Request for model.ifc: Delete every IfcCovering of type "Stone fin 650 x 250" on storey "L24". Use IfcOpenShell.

First a look at what the model holds.

```python
import ifcopenshell
import ifcopenshell.util.element

model = ifcopenshell.open("model.ifc")
print(model.schema)
storey = next(s for s in model.by_type("IfcBuildingStorey") if s.Name == "L24")
coverings = [e for e in ifcopenshell.util.element.get_decomposition(storey) if e.is_a("IfcCovering")]
seen = {}
for e in coverings:
    element_type = ifcopenshell.util.element.get_type(e)
    name = element_type.Name if element_type not in (None, e) else None
    seen[name] = seen.get(name, 0) + 1
for name, count in sorted(seen.items(), key=str):
    print(count, "x", name)
```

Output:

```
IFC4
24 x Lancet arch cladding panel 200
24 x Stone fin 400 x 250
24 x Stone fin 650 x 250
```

```python
import ifcopenshell
import ifcopenshell.api.root
import ifcopenshell.util.element

model = ifcopenshell.open("model.ifc")

storey = next(s for s in model.by_type("IfcBuildingStorey") if s.Name == "L24")
coverings = [e for e in ifcopenshell.util.element.get_decomposition(storey) if e.is_a("IfcCovering")]
targets = [e for e in coverings if (t := ifcopenshell.util.element.get_type(e)) not in (None, e) and t.Name == "Stone fin 650 x 250"]

for e in targets:
    ifcopenshell.api.root.remove_product(model, product=e)
print(len(targets), "removed")

model.write("model-out.ifc")
```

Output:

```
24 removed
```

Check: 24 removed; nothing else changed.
